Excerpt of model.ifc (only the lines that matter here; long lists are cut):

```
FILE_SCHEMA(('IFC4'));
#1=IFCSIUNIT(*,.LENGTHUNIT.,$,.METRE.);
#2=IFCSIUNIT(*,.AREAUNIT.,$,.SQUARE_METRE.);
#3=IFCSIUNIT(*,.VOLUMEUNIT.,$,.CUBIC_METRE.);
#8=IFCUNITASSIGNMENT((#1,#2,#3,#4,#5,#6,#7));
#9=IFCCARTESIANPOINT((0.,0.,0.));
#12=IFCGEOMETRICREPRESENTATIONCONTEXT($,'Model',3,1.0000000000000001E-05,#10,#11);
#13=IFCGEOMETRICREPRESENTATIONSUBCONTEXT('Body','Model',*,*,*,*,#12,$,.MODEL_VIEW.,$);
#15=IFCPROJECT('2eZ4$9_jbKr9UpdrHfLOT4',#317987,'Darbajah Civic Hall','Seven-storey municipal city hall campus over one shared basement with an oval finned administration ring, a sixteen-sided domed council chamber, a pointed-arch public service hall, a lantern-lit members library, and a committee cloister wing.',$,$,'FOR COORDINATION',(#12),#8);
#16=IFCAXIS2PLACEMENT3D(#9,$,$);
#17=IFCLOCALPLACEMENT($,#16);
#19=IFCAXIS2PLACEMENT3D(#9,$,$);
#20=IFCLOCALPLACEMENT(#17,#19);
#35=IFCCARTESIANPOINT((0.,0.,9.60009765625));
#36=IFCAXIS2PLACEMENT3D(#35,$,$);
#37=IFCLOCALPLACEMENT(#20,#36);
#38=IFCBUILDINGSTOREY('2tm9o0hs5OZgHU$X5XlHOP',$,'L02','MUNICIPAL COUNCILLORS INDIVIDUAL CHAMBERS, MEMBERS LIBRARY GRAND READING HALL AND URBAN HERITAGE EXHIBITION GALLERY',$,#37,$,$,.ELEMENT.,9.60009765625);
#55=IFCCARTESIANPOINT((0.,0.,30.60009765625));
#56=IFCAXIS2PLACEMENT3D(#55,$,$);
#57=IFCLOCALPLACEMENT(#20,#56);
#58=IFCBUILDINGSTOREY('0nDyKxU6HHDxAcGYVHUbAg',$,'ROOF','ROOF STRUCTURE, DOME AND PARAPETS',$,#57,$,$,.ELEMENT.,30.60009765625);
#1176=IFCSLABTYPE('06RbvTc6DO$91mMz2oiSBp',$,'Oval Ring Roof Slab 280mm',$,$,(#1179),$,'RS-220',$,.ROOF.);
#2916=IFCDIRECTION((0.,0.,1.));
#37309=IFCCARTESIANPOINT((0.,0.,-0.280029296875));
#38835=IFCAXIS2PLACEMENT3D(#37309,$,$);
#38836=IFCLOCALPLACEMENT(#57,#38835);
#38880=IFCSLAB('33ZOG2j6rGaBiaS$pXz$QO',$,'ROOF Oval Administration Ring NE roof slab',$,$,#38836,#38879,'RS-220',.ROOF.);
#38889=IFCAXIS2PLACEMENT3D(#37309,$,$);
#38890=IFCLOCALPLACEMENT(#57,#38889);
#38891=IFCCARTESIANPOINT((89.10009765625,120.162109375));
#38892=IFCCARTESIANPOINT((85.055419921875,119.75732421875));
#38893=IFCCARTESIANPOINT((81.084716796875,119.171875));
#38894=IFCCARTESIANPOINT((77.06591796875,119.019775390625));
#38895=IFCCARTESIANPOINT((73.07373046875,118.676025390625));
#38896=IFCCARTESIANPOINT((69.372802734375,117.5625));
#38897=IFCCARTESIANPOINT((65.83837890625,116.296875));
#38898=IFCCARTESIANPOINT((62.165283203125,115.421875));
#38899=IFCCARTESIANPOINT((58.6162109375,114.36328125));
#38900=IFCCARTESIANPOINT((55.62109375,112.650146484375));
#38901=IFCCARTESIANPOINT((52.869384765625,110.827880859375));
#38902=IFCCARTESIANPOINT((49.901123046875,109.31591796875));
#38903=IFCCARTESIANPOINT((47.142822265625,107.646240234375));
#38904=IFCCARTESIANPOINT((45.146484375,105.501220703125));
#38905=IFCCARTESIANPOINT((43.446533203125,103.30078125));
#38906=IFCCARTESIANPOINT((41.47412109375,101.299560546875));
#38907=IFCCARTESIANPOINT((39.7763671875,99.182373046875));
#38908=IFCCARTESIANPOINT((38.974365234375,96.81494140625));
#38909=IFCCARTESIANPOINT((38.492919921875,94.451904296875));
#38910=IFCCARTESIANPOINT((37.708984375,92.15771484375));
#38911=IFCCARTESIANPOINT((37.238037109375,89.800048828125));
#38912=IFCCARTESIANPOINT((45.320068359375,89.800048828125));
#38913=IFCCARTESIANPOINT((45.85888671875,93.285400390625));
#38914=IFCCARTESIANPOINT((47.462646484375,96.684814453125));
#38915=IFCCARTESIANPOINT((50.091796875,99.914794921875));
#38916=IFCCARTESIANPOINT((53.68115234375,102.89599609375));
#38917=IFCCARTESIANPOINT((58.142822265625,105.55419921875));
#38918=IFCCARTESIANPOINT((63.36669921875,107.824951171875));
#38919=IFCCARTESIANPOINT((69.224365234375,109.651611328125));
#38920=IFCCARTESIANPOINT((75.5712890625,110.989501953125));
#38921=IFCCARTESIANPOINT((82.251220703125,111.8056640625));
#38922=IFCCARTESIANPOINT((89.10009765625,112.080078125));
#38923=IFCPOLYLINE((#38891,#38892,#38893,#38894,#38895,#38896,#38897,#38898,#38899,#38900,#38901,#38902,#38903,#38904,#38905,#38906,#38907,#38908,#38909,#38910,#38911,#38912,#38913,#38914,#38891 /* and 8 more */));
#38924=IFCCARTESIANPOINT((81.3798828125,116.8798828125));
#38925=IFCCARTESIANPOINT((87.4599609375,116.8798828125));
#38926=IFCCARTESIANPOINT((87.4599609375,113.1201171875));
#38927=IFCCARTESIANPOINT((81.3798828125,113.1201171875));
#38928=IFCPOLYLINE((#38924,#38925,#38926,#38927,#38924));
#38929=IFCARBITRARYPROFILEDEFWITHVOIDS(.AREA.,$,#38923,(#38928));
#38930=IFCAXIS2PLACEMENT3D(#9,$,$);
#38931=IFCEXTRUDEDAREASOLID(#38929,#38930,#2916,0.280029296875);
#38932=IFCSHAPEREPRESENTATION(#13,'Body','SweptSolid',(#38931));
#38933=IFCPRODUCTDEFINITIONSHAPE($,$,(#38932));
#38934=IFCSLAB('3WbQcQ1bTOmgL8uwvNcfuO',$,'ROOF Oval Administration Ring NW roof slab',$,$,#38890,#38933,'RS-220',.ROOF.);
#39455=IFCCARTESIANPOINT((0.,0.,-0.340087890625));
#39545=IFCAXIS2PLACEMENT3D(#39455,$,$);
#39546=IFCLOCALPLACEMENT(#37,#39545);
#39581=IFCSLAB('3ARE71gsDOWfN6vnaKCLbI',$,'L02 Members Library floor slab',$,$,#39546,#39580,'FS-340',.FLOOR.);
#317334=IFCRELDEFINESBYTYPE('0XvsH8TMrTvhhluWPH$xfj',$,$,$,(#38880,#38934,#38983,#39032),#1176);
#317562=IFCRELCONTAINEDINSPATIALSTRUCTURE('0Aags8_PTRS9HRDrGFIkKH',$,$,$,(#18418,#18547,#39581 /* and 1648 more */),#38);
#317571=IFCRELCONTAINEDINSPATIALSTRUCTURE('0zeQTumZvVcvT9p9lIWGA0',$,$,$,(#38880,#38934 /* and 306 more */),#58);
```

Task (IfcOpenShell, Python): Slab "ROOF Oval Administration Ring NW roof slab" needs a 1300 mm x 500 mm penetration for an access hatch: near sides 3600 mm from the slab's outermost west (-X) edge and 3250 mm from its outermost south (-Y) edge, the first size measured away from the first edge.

```python
import numpy as np
import ifcopenshell
import ifcopenshell.api.feature
import ifcopenshell.api.geometry
import ifcopenshell.api.root
import ifcopenshell.geom
import ifcopenshell.util.placement
import ifcopenshell.util.representation
import ifcopenshell.util.shape
import ifcopenshell.util.unit

model = ifcopenshell.open("model.ifc")
unit_scale = ifcopenshell.util.unit.calculate_unit_scale(model)
settings = ifcopenshell.geom.settings()


def volume(element):
    """Net volume in cubic metres, openings subtracted."""
    shape = ifcopenshell.geom.create_shape(settings, element)
    return ifcopenshell.util.shape.get_volume(shape.geometry)


slab = model.by_guid("3WbQcQ1bTOmgL8uwvNcfuO")
before = volume(slab)

# Extent in the slab's own axes, in metres. The edges named are its -X and -Y sides.
slab_shape = ifcopenshell.geom.create_shape(settings, slab)
vertices = ifcopenshell.util.shape.get_vertices(slab_shape.geometry)
x_min, y_min, bottom = vertices.min(axis=0)
top = vertices[:, 2].max()

opening = ifcopenshell.api.root.create_entity(model, ifc_class="IfcOpeningElement", name="Access hatch opening", predefined_type="OPENING")
context = ifcopenshell.util.representation.get_context(model, "Model", "Body", "MODEL_VIEW")
width, depth = 1.3, 0.5
outline = [(0.0, 0.0), (width, 0.0), (width, depth), (0.0, depth), (0.0, 0.0)]
# Overshoot both faces by 50 mm so the cut is clean.
shape = ifcopenshell.api.geometry.add_slab_representation(
    model, context=context, depth=top - bottom + 0.1, polyline=outline
)
ifcopenshell.api.geometry.assign_representation(model, product=opening, representation=shape)

matrix = ifcopenshell.util.placement.get_local_placement(slab.ObjectPlacement)
matrix[:, 3] = matrix @ np.append(np.array([x_min + 3.6, y_min + 3.25, bottom - 0.05]) / unit_scale, 1.0)
ifcopenshell.api.geometry.edit_object_placement(model, product=opening, matrix=matrix, is_si=False)
ifcopenshell.api.feature.add_feature(model, feature=opening, element=slab)

after = volume(slab)

print(f"slab volume {before:.3f} -> {after:.3f} m3")

model.write("model-out.ifc")
```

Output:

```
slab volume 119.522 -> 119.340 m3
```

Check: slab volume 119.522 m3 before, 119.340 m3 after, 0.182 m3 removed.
